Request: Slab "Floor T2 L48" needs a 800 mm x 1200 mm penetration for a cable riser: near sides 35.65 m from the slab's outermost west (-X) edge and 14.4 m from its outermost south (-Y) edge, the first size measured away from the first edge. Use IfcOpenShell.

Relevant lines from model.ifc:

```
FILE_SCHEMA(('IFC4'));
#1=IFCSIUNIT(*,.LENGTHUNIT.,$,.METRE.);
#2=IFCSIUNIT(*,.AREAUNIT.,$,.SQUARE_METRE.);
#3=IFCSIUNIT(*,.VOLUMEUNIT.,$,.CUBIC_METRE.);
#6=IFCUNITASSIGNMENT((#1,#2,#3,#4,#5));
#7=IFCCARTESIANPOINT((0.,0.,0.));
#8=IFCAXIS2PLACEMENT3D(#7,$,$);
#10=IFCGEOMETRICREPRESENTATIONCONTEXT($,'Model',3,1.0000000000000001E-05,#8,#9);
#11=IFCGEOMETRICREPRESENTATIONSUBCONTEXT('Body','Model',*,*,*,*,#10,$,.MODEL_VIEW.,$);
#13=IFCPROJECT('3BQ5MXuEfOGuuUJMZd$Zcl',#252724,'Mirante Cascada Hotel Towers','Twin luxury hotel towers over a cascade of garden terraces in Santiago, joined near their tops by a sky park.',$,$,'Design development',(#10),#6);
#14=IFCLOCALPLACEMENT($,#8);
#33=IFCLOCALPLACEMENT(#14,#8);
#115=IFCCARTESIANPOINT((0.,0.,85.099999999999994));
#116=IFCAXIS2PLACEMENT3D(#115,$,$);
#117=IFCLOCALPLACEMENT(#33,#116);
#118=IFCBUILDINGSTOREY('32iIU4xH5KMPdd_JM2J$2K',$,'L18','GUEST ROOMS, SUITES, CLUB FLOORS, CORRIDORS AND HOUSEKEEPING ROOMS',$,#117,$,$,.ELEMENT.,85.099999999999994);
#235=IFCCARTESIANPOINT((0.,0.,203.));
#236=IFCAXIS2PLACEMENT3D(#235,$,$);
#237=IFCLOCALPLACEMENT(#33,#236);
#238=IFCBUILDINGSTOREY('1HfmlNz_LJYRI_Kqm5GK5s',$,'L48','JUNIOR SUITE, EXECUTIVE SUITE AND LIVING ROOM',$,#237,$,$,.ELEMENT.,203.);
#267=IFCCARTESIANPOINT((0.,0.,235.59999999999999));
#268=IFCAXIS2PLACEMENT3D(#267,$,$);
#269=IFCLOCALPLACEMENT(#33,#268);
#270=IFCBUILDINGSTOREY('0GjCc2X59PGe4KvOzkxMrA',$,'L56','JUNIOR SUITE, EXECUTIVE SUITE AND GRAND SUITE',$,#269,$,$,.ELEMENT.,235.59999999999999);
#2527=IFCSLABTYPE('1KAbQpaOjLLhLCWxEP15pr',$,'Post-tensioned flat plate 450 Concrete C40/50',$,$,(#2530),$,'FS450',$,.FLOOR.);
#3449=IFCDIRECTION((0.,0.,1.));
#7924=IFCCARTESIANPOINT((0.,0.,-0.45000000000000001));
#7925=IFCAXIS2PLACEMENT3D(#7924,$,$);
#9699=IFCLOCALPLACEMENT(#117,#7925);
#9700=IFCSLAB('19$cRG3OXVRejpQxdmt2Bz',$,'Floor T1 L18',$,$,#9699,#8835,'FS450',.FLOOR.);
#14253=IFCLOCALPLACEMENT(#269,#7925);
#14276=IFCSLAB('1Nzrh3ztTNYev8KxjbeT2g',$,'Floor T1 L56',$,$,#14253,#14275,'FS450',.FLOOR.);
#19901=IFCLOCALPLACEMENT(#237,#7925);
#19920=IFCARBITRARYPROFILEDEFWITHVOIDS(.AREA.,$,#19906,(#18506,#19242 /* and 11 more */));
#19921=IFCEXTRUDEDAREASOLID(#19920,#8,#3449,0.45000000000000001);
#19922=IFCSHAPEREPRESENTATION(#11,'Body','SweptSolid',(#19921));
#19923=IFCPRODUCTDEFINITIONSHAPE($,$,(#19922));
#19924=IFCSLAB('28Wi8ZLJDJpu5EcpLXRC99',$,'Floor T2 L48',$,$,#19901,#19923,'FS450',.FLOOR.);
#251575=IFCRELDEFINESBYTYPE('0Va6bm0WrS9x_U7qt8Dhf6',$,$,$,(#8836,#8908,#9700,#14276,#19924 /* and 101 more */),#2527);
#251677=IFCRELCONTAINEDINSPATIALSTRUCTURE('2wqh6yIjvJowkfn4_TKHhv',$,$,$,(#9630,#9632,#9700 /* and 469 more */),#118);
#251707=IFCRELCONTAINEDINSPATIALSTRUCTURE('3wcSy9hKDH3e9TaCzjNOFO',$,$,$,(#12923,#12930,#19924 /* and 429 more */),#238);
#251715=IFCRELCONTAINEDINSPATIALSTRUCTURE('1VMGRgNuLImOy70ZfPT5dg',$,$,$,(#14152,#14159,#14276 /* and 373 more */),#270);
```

```python
import numpy as np
import ifcopenshell
import ifcopenshell.api.feature
import ifcopenshell.api.geometry
import ifcopenshell.api.root
import ifcopenshell.geom
import ifcopenshell.util.placement
import ifcopenshell.util.representation
import ifcopenshell.util.shape
import ifcopenshell.util.unit

model = ifcopenshell.open("model.ifc")
unit_scale = ifcopenshell.util.unit.calculate_unit_scale(model)
settings = ifcopenshell.geom.settings()


def volume(element):
    """Net volume in cubic metres, openings subtracted."""
    shape = ifcopenshell.geom.create_shape(settings, element)
    return ifcopenshell.util.shape.get_volume(shape.geometry)


slab = model.by_guid("28Wi8ZLJDJpu5EcpLXRC99")
before = volume(slab)

# Extent in the slab's own axes, in metres. The edges named are its -X and -Y sides.
slab_shape = ifcopenshell.geom.create_shape(settings, slab)
vertices = ifcopenshell.util.shape.get_vertices(slab_shape.geometry)
x_min, y_min, bottom = vertices.min(axis=0)
top = vertices[:, 2].max()

opening = ifcopenshell.api.root.create_entity(model, ifc_class="IfcOpeningElement", name="Cable riser opening", predefined_type="OPENING")
context = ifcopenshell.util.representation.get_context(model, "Model", "Body", "MODEL_VIEW")
width, depth = 0.8, 1.2
outline = [(0.0, 0.0), (width, 0.0), (width, depth), (0.0, depth), (0.0, 0.0)]
# Overshoot both faces by 50 mm so the cut is clean.
shape = ifcopenshell.api.geometry.add_slab_representation(
    model, context=context, depth=top - bottom + 0.1, polyline=outline
)
ifcopenshell.api.geometry.assign_representation(model, product=opening, representation=shape)

matrix = ifcopenshell.util.placement.get_local_placement(slab.ObjectPlacement)
matrix[:, 3] = matrix @ np.append(np.array([x_min + 35.65, y_min + 14.4, bottom - 0.05]) / unit_scale, 1.0)
ifcopenshell.api.geometry.edit_object_placement(model, product=opening, matrix=matrix, is_si=False)
ifcopenshell.api.feature.add_feature(model, feature=opening, element=slab)

after = volume(slab)

print(f"slab volume {before:.3f} -> {after:.3f} m3")

model.write("model_v2.ifc")
```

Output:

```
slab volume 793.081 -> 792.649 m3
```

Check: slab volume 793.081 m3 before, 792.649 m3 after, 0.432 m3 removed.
